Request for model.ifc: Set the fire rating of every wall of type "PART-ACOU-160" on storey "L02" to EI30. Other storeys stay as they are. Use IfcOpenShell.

First a look at what the model holds.

```python
import ifcopenshell
import ifcopenshell.util.element

model = ifcopenshell.open("model.ifc")
print(model.schema)
storey = next(s for s in model.by_type("IfcBuildingStorey") if s.Name == "L02")
walls = [e for e in ifcopenshell.util.element.get_decomposition(storey) if e.is_a("IfcWall")]
seen = {}
for e in walls:
    element_type = ifcopenshell.util.element.get_type(e)
    key = (element_type.Name if element_type != e and element_type else None, ifcopenshell.util.element.get_pset(e, "Pset_WallCommon", "FireRating"))
    seen[key] = seen.get(key, 0) + 1
for (name, value), count in sorted(seen.items(), key=str):
    print(count, "x", name, "|", value)
```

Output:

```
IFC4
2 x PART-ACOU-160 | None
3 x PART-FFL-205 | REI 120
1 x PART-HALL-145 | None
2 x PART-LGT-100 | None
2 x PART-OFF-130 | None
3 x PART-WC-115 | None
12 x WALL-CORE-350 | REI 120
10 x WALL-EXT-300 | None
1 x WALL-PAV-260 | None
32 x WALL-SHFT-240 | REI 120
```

```python
import ifcopenshell
import ifcopenshell.api.pset
import ifcopenshell.util.element

model = ifcopenshell.open("model.ifc")

storey = next(s for s in model.by_type("IfcBuildingStorey") if s.Name == "L02")
walls = [e for e in ifcopenshell.util.element.get_decomposition(storey) if e.is_a("IfcWall")]

count = 0
for e in walls:
    element_type = ifcopenshell.util.element.get_type(e)
    if element_type in (None, e) or element_type.Name != "PART-ACOU-160":
        continue
    # add_pset returns the element's existing set when there is one.
    pset = ifcopenshell.api.pset.add_pset(model, product=e, name="Pset_WallCommon")
    ifcopenshell.api.pset.edit_pset(model, pset=pset, properties={"FireRating": "EI30"})
    count += 1

print(count, "walls updated")

model.write("model-out.ifc")
```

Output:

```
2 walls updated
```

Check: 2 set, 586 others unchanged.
